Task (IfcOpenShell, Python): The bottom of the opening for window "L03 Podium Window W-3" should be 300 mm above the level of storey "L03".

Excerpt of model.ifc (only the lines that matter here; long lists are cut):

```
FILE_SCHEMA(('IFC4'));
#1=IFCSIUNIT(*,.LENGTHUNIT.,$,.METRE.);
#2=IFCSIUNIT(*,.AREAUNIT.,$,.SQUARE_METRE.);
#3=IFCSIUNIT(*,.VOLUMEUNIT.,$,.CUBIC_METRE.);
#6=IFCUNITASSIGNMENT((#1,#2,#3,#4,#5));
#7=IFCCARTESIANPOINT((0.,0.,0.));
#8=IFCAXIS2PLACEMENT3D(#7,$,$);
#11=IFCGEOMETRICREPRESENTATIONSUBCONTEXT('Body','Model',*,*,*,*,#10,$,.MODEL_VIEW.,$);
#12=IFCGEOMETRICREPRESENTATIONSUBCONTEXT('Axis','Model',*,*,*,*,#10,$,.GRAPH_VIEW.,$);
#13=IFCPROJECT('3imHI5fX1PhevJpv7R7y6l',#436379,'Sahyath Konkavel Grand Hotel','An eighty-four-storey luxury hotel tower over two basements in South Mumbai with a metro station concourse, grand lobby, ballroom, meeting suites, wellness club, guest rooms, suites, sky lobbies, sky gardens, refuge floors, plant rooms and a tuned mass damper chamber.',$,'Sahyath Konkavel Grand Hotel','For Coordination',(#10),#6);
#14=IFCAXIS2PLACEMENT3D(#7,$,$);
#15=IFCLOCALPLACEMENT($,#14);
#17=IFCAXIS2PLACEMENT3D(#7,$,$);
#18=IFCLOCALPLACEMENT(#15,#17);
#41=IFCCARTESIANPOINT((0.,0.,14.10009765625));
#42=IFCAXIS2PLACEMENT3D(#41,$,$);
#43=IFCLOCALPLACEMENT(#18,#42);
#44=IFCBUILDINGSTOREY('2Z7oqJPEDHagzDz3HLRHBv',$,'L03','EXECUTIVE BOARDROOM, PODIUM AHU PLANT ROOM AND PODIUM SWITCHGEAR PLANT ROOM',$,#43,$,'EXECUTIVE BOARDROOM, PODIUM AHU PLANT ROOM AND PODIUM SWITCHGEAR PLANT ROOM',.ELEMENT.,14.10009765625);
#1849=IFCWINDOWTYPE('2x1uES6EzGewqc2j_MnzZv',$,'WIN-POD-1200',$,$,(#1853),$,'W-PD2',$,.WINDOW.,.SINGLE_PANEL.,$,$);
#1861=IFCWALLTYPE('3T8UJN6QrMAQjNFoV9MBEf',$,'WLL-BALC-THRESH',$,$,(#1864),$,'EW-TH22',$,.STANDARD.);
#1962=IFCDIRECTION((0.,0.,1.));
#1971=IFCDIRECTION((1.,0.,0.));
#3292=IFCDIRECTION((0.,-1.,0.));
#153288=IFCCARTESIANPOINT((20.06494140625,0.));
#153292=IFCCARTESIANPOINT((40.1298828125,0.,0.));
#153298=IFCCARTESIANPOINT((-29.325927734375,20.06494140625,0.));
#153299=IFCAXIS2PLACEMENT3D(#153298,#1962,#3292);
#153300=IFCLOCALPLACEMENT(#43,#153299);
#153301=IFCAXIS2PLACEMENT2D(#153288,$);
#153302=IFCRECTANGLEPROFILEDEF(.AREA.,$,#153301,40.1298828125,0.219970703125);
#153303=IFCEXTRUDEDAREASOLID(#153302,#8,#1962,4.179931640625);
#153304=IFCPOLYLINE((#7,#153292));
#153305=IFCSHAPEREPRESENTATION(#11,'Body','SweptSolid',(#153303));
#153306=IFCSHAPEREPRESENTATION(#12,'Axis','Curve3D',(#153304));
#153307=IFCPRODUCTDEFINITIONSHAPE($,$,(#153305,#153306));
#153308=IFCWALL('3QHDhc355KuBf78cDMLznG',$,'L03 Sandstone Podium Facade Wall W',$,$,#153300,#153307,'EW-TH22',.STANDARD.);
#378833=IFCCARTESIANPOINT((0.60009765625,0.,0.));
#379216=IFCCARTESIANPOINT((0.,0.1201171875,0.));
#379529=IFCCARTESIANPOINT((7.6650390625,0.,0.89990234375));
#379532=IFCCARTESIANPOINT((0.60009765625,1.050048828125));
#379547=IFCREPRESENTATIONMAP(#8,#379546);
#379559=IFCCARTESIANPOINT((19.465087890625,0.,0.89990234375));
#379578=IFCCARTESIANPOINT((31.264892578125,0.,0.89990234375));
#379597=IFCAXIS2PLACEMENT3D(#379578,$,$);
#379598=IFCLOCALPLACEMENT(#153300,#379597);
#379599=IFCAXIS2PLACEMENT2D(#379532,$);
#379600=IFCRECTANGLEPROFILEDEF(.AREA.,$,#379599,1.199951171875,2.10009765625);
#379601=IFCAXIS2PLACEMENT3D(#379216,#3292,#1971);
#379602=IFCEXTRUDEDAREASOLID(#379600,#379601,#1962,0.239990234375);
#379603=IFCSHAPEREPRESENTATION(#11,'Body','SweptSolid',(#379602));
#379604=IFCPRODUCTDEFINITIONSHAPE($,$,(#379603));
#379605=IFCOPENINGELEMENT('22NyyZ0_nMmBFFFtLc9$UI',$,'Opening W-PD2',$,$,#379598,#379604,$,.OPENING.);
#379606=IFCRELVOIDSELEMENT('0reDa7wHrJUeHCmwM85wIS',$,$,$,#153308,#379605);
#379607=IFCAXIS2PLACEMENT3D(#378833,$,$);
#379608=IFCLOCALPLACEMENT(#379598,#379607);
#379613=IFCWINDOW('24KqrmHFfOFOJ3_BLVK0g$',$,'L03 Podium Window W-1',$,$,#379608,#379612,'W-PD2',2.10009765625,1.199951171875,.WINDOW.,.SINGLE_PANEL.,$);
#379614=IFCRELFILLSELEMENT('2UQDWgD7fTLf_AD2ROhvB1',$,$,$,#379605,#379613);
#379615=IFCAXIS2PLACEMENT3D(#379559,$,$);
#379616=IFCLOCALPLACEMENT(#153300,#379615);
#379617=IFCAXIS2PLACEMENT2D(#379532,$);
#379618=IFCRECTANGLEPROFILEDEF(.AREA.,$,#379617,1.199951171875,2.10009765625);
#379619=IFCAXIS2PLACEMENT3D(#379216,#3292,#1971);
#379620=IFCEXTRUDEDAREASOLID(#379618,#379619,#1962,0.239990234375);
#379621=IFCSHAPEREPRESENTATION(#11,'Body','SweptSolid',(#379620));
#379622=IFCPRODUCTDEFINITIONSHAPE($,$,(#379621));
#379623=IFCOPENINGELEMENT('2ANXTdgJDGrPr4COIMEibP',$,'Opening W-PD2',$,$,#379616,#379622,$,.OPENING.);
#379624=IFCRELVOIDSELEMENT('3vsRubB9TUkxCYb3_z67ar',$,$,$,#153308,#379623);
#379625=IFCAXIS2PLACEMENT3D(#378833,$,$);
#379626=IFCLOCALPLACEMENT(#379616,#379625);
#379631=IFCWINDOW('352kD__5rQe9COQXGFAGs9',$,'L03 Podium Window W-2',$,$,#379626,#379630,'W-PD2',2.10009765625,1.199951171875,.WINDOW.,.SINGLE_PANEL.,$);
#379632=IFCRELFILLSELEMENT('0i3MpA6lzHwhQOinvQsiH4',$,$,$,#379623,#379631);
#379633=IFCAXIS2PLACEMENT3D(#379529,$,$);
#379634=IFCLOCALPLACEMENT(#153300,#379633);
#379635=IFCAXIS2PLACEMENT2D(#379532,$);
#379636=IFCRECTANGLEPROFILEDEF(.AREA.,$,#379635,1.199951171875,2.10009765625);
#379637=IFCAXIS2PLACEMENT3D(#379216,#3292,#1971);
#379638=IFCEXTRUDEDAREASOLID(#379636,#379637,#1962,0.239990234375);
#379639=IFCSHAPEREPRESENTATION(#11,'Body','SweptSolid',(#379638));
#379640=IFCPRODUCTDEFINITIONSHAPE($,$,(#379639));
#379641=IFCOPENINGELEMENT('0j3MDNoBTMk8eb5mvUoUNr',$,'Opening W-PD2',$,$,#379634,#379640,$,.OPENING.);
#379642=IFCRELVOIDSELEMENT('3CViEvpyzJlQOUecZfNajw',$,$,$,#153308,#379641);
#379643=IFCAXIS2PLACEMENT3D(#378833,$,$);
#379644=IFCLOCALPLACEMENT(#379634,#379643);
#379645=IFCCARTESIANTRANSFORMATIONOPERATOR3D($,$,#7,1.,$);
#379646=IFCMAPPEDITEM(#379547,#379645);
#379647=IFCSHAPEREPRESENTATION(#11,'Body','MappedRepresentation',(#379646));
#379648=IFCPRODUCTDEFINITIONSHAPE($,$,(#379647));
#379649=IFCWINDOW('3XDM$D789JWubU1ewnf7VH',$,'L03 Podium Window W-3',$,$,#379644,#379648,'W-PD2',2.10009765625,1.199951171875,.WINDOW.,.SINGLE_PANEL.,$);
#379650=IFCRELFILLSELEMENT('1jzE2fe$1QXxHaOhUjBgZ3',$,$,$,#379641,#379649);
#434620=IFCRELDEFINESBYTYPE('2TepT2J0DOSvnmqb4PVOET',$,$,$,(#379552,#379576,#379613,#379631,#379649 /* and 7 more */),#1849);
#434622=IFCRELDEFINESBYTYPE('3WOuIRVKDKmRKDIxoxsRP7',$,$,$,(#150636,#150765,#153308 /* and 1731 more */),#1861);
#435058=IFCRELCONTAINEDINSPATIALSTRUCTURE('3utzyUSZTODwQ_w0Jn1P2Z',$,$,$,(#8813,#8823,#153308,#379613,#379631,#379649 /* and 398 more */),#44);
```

```python
import numpy as np
import ifcopenshell
import ifcopenshell.api.geometry
import ifcopenshell.geom
import ifcopenshell.util.element
import ifcopenshell.util.placement
import ifcopenshell.util.shape
import ifcopenshell.util.unit

model = ifcopenshell.open("model.ifc")
unit_scale = ifcopenshell.util.unit.calculate_unit_scale(model)

window = model.by_guid("3XDM$D789JWubU1ewnf7VH")
opening = window.FillsVoids[0].RelatingOpeningElement
storey = ifcopenshell.util.element.get_container(window, ifc_class="IfcBuildingStorey")
level = ifcopenshell.util.placement.get_local_placement(storey.ObjectPlacement)[2, 3]

# The opening's origin need not be at the sill, so measure its lowest point.
shape = ifcopenshell.geom.create_shape(ifcopenshell.geom.settings(), opening)
bottom = ifcopenshell.util.shape.get_shape_bottom_elevation(shape, shape.geometry) / unit_scale
dz = level + 0.3 - bottom

shift = np.array([0.0, 0.0, dz])
# The window is placed relative to its opening, so it follows when the opening moves.
matrix = ifcopenshell.util.placement.get_local_placement(opening.ObjectPlacement)
matrix[:3, 3] += shift
ifcopenshell.api.geometry.edit_object_placement(
    model, product=opening, matrix=matrix, is_si=False, should_transform_children=True
)

print(f"moved by {dz * unit_scale:+.3f} m")

model.write("model_edited.ifc")
```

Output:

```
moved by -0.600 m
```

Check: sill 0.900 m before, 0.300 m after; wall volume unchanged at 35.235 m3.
